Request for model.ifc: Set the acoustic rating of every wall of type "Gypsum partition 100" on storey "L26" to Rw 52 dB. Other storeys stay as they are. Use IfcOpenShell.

First a look at what the model holds.

```python
import ifcopenshell
import ifcopenshell.util.element

model = ifcopenshell.open("model.ifc")
print(model.schema)
storey = next(s for s in model.by_type("IfcBuildingStorey") if s.Name == "L26")
walls = [e for e in ifcopenshell.util.element.get_decomposition(storey) if e.is_a("IfcWall")]
seen = {}
for e in walls:
    element_type = ifcopenshell.util.element.get_type(e)
    key = (element_type.Name if element_type != e and element_type else None, ifcopenshell.util.element.get_pset(e, "Pset_WallCommon", "AcousticRating"))
    seen[key] = seen.get(key, 0) + 1
for (name, value), count in sorted(seen.items(), key=str):
    print(count, "x", name, "|", value)
```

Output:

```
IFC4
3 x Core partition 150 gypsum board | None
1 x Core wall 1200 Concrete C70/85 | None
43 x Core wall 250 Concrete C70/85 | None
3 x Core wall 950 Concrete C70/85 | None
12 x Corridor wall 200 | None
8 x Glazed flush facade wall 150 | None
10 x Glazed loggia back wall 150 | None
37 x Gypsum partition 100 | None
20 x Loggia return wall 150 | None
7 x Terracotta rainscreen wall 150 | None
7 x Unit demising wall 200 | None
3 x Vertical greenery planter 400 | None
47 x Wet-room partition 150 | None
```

```python
import ifcopenshell
import ifcopenshell.api.pset
import ifcopenshell.util.element

model = ifcopenshell.open("model.ifc")

storey = next(s for s in model.by_type("IfcBuildingStorey") if s.Name == "L26")
walls = [e for e in ifcopenshell.util.element.get_decomposition(storey) if e.is_a("IfcWall")]

count = 0
for e in walls:
    element_type = ifcopenshell.util.element.get_type(e)
    if element_type in (None, e) or element_type.Name != "Gypsum partition 100":
        continue
    found = ifcopenshell.util.element.get_pset(e, "Pset_WallCommon", should_inherit=False)
    if found:
        pset = model.by_id(found["id"])
        if len(ifcopenshell.util.element.get_elements_by_pset(pset)) > 1:
            pset = ifcopenshell.api.pset.unshare_pset(model, products=[e], pset=pset)[0]
    else:
        pset = ifcopenshell.api.pset.add_pset(model, product=e, name="Pset_WallCommon")
    ifcopenshell.api.pset.edit_pset(model, pset=pset, properties={"AcousticRating": "Rw 52 dB"})
    count += 1

print(count, "walls updated")

model.write("model_rev.ifc")
```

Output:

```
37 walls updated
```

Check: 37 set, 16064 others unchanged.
